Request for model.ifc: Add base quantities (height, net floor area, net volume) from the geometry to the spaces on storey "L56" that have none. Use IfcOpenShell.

First a look at what the model holds.

```python
import ifcopenshell
import ifcopenshell.util.element
import ifcopenshell.util.unit

model = ifcopenshell.open("model.ifc")
print(model.schema)
for unit_type in ("LENGTHUNIT", "AREAUNIT", "VOLUMEUNIT"):
    print(unit_type, ifcopenshell.util.unit.calculate_unit_scale(model, unit_type))
storey = next(s for s in model.by_type("IfcBuildingStorey") if s.Name == "L56")
spaces = [e for e in ifcopenshell.util.element.get_decomposition(storey) if e.is_a("IfcSpace")]
for e in sorted(spaces, key=lambda e: e.id()):
    print(e.id(), e.is_a(), e.Name, list(ifcopenshell.util.element.get_psets(e, qtos_only=True)), sep=" | ")
```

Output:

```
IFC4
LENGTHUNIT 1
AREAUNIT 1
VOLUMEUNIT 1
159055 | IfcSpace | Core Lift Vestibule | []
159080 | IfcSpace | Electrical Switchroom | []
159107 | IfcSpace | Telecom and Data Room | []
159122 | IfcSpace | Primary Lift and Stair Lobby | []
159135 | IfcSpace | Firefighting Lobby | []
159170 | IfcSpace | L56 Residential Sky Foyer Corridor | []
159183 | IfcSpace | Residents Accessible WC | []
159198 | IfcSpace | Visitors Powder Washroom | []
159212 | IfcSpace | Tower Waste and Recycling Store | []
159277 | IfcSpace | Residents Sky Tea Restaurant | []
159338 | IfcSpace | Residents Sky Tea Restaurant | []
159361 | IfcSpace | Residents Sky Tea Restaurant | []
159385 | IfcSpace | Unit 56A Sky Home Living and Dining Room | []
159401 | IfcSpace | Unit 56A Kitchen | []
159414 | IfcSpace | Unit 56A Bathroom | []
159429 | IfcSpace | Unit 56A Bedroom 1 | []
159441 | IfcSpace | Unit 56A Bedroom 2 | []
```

```python
import ifcopenshell
import ifcopenshell.api.pset
import ifcopenshell.geom
import ifcopenshell.util.element
import ifcopenshell.util.shape
import ifcopenshell.util.unit

model = ifcopenshell.open("model.ifc")
unit_scale = ifcopenshell.util.unit.calculate_unit_scale(model)
area_scale = ifcopenshell.util.unit.calculate_unit_scale(model, "AREAUNIT")
volume_scale = ifcopenshell.util.unit.calculate_unit_scale(model, "VOLUMEUNIT")
settings = ifcopenshell.geom.settings()

storey = next(s for s in model.by_type("IfcBuildingStorey") if s.Name == "L56")
spaces = [e for e in ifcopenshell.util.element.get_decomposition(storey) if e.is_a("IfcSpace")]

for e in sorted(spaces, key=lambda e: e.id()):
    if ifcopenshell.util.element.get_psets(e, qtos_only=True, should_inherit=False):
        continue
    # Geometry comes back in metres, in the element's own axes.
    shape = ifcopenshell.geom.create_shape(settings, e)
    values = {
        "Height": ifcopenshell.util.shape.get_z(shape.geometry) / unit_scale,
        "NetFloorArea": ifcopenshell.util.shape.get_footprint_area(shape.geometry) / area_scale,
        "NetVolume": ifcopenshell.util.shape.get_volume(shape.geometry) / volume_scale,
    }
    qto = ifcopenshell.api.pset.add_qto(model, product=e, name="Qto_SpaceBaseQuantities")
    ifcopenshell.api.pset.edit_qto(model, qto=qto, properties=values)
    print(e.id(), {k: round(v, 3) for k, v in values.items()})

model.write("model_updated.ifc")
```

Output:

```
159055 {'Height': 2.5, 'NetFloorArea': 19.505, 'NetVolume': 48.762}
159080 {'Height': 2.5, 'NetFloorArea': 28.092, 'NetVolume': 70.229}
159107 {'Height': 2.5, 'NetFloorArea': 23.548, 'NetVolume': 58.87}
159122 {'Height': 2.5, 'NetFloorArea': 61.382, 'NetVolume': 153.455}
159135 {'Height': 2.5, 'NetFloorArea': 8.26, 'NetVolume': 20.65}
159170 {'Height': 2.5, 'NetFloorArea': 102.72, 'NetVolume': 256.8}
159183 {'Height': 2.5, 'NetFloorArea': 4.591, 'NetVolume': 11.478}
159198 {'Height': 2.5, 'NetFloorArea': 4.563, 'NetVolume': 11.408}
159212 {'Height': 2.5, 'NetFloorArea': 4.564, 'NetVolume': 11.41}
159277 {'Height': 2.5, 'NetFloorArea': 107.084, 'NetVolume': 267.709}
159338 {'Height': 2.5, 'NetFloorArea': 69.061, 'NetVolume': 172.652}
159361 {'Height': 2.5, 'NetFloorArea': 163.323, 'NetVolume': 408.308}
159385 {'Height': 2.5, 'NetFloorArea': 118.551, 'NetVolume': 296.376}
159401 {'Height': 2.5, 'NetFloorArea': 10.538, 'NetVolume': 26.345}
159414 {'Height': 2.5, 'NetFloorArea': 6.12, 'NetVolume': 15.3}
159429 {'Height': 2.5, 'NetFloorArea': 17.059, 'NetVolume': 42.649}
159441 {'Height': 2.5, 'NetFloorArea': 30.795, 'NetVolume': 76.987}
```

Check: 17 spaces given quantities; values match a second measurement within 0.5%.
